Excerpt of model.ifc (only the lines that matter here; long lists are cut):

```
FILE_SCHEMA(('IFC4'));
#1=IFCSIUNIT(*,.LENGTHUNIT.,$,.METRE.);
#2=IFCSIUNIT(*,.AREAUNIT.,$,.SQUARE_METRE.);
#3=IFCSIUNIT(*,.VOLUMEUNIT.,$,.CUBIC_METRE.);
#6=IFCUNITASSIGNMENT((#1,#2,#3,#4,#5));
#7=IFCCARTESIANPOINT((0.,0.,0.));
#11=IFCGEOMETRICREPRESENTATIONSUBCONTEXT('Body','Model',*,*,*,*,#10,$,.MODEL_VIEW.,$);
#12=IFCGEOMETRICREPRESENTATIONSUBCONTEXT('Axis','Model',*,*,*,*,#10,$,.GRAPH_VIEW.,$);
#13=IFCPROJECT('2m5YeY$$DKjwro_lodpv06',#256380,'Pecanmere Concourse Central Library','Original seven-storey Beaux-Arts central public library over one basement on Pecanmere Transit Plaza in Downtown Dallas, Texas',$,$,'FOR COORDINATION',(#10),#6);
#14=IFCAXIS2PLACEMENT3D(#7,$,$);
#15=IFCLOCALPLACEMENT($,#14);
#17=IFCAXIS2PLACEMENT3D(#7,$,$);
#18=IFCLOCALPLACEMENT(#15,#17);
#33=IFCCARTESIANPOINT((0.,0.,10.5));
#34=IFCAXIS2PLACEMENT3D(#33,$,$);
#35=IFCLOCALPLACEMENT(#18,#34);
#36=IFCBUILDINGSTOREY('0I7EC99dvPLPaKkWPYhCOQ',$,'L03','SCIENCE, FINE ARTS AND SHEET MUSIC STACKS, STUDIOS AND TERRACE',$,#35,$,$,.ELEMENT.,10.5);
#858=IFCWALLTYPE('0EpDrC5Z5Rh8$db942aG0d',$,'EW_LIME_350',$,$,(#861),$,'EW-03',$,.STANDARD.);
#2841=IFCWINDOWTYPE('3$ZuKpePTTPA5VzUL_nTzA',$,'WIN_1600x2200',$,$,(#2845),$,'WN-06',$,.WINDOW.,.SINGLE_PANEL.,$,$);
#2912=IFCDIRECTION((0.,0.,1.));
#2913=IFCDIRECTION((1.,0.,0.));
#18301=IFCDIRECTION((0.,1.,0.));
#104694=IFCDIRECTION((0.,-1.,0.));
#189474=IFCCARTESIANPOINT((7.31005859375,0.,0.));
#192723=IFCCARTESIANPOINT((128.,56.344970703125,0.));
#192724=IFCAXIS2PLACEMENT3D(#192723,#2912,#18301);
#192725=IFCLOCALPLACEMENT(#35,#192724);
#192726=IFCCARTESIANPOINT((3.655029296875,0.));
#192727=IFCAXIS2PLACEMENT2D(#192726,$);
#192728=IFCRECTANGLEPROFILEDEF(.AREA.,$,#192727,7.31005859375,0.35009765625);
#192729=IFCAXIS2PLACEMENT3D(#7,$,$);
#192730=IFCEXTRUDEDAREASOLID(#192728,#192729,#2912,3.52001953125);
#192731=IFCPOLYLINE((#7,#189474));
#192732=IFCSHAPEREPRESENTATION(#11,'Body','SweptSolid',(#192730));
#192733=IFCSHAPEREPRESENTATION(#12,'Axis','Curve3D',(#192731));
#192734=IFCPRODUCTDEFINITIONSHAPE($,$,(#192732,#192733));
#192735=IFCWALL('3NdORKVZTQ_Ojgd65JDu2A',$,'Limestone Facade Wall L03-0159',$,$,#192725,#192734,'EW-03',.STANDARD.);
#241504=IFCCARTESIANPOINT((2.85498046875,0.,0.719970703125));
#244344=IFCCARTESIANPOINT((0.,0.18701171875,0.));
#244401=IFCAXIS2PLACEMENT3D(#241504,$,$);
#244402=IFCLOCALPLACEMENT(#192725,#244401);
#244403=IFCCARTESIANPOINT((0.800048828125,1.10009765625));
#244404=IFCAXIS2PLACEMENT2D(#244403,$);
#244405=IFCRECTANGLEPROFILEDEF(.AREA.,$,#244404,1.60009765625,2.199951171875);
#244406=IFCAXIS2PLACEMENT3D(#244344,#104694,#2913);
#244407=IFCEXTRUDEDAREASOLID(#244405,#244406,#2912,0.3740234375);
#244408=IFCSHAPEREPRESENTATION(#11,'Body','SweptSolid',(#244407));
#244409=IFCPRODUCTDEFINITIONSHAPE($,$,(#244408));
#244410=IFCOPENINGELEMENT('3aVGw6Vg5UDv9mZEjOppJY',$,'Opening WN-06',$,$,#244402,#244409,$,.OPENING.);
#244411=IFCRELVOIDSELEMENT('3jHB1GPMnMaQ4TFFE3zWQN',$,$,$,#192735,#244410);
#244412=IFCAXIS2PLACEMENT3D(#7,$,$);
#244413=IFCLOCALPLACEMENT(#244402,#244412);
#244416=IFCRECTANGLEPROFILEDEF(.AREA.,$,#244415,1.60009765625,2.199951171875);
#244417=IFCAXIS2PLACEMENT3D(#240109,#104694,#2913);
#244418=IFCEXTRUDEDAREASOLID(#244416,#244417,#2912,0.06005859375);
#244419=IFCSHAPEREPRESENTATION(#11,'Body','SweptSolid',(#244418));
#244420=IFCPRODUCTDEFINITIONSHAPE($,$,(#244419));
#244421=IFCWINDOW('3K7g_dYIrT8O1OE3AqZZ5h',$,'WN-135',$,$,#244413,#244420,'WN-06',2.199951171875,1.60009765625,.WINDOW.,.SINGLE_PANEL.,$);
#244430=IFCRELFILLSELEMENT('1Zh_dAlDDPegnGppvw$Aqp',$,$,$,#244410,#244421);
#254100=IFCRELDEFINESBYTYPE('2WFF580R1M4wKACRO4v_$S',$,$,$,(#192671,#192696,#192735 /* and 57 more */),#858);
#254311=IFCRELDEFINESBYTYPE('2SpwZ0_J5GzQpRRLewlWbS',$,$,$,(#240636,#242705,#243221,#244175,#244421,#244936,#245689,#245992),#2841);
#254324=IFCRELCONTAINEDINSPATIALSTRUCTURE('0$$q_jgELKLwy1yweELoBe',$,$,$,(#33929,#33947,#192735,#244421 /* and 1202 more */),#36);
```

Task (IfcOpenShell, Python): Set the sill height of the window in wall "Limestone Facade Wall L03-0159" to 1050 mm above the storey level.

```python
import numpy as np
import ifcopenshell
import ifcopenshell.api.geometry
import ifcopenshell.geom
import ifcopenshell.util.element
import ifcopenshell.util.placement
import ifcopenshell.util.shape
import ifcopenshell.util.unit

model = ifcopenshell.open("model.ifc")
unit_scale = ifcopenshell.util.unit.calculate_unit_scale(model)

window = model.by_id(244421)
opening = window.FillsVoids[0].RelatingOpeningElement
storey = ifcopenshell.util.element.get_container(window, ifc_class="IfcBuildingStorey")
level = ifcopenshell.util.placement.get_local_placement(storey.ObjectPlacement)[2, 3]

# The opening's origin need not be at the sill, so measure its lowest point.
shape = ifcopenshell.geom.create_shape(ifcopenshell.geom.settings(), opening)
bottom = ifcopenshell.util.shape.get_shape_bottom_elevation(shape, shape.geometry) / unit_scale
dz = level + 1.05 / unit_scale - bottom

shift = np.array([0.0, 0.0, dz])
# The window is placed relative to its opening, so it follows when the opening moves.
matrix = ifcopenshell.util.placement.get_local_placement(opening.ObjectPlacement)
matrix[:3, 3] += shift
ifcopenshell.api.geometry.edit_object_placement(
    model, product=opening, matrix=matrix, is_si=False, should_transform_children=True
)

print(f"moved by {dz * unit_scale:+.3f} m")

model.write("model_updated.ifc")
```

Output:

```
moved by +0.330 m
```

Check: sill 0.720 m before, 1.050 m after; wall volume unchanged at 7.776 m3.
